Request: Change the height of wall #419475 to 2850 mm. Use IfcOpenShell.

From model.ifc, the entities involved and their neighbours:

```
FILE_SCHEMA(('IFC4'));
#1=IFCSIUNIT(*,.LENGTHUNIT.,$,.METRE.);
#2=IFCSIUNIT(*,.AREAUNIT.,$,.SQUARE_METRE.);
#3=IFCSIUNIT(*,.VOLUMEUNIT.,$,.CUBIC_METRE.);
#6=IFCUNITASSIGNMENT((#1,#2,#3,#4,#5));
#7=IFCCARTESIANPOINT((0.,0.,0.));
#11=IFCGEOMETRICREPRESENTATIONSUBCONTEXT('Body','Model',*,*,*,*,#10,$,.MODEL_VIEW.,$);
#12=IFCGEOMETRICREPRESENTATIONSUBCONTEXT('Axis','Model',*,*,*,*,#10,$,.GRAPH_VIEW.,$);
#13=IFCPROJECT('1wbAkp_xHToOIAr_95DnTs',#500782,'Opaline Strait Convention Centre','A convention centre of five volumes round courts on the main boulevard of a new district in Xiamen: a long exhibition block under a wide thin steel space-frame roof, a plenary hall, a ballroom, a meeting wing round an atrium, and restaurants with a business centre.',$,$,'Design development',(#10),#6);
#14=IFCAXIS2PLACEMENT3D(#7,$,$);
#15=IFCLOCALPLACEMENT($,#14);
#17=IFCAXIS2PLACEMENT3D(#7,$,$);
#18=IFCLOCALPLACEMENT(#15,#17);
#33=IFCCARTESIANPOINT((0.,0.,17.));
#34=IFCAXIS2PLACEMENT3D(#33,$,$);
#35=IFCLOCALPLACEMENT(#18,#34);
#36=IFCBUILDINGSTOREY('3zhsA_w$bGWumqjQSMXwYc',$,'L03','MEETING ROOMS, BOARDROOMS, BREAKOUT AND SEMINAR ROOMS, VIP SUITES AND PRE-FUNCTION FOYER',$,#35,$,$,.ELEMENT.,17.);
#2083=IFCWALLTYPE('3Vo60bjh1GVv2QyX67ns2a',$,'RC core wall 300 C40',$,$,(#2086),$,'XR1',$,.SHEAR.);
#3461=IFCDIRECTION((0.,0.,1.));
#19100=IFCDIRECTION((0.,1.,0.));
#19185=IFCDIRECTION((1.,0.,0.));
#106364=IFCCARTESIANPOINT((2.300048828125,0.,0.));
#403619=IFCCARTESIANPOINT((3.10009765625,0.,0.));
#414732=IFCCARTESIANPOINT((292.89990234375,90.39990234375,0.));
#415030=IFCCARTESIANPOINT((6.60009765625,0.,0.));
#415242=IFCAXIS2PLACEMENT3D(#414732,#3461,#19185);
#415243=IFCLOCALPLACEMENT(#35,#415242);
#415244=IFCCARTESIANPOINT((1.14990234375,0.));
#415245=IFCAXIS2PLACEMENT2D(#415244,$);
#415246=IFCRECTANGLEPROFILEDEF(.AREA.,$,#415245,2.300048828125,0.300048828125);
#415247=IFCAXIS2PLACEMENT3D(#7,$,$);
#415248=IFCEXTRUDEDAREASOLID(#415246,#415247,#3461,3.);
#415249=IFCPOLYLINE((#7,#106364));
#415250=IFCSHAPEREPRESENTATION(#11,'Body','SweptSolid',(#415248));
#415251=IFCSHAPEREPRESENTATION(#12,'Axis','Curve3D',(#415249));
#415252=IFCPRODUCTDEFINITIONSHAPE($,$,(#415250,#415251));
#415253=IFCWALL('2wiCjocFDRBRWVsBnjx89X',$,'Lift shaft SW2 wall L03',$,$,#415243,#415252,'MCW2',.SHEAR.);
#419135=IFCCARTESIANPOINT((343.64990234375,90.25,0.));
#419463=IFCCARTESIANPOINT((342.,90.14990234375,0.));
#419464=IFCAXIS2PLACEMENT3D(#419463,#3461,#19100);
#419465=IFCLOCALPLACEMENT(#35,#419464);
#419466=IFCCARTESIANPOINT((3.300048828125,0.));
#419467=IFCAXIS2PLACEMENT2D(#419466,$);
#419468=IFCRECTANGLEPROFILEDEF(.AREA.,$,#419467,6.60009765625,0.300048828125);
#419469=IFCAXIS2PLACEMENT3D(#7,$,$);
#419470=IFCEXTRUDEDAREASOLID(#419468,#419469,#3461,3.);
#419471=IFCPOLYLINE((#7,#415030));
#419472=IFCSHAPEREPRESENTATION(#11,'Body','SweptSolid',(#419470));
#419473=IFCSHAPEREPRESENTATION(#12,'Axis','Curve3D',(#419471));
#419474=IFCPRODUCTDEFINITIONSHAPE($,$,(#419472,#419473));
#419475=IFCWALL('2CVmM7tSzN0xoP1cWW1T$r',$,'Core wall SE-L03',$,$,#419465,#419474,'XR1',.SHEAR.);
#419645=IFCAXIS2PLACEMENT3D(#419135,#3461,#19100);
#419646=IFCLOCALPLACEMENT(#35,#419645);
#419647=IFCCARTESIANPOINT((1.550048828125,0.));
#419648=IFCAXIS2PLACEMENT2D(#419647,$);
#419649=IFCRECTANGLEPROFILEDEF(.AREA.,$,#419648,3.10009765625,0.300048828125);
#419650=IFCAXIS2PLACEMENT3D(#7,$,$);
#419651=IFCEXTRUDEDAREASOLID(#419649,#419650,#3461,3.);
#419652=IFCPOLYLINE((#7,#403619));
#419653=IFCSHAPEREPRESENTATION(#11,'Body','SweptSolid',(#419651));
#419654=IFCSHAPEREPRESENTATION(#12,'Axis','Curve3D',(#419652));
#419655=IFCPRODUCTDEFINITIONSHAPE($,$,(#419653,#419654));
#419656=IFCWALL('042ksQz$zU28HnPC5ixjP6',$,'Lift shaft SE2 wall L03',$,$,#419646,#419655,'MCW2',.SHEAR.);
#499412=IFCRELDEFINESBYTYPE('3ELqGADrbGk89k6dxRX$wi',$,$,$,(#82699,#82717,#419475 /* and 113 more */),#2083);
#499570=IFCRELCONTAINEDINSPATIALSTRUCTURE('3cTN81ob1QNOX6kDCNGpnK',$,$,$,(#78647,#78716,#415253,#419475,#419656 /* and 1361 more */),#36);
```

```python
import ifcopenshell
import ifcopenshell.geom
import ifcopenshell.util.representation
import ifcopenshell.util.shape
import ifcopenshell.util.unit

model = ifcopenshell.open("model.ifc")
unit_scale = ifcopenshell.util.unit.calculate_unit_scale(model)
settings = ifcopenshell.geom.settings()


def volume(element):
    """Net volume in cubic metres, openings subtracted."""
    shape = ifcopenshell.geom.create_shape(settings, element)
    return ifcopenshell.util.shape.get_volume(shape.geometry)


wall = model.by_guid("2CVmM7tSzN0xoP1cWW1T$r")
before = volume(wall)

body = ifcopenshell.util.representation.get_representation(wall, "Model", "Body")
solid = body.Items[0]
old_height = solid.Depth
solid.Depth = 2.85 / unit_scale
after = volume(wall)

print(f"height {old_height:g} -> {solid.Depth:g}, volume {before:.3f} -> {after:.3f} m3")

model.write("model_v2.ifc")
```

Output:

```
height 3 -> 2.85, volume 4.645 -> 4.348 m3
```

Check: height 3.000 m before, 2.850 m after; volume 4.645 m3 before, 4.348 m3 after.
